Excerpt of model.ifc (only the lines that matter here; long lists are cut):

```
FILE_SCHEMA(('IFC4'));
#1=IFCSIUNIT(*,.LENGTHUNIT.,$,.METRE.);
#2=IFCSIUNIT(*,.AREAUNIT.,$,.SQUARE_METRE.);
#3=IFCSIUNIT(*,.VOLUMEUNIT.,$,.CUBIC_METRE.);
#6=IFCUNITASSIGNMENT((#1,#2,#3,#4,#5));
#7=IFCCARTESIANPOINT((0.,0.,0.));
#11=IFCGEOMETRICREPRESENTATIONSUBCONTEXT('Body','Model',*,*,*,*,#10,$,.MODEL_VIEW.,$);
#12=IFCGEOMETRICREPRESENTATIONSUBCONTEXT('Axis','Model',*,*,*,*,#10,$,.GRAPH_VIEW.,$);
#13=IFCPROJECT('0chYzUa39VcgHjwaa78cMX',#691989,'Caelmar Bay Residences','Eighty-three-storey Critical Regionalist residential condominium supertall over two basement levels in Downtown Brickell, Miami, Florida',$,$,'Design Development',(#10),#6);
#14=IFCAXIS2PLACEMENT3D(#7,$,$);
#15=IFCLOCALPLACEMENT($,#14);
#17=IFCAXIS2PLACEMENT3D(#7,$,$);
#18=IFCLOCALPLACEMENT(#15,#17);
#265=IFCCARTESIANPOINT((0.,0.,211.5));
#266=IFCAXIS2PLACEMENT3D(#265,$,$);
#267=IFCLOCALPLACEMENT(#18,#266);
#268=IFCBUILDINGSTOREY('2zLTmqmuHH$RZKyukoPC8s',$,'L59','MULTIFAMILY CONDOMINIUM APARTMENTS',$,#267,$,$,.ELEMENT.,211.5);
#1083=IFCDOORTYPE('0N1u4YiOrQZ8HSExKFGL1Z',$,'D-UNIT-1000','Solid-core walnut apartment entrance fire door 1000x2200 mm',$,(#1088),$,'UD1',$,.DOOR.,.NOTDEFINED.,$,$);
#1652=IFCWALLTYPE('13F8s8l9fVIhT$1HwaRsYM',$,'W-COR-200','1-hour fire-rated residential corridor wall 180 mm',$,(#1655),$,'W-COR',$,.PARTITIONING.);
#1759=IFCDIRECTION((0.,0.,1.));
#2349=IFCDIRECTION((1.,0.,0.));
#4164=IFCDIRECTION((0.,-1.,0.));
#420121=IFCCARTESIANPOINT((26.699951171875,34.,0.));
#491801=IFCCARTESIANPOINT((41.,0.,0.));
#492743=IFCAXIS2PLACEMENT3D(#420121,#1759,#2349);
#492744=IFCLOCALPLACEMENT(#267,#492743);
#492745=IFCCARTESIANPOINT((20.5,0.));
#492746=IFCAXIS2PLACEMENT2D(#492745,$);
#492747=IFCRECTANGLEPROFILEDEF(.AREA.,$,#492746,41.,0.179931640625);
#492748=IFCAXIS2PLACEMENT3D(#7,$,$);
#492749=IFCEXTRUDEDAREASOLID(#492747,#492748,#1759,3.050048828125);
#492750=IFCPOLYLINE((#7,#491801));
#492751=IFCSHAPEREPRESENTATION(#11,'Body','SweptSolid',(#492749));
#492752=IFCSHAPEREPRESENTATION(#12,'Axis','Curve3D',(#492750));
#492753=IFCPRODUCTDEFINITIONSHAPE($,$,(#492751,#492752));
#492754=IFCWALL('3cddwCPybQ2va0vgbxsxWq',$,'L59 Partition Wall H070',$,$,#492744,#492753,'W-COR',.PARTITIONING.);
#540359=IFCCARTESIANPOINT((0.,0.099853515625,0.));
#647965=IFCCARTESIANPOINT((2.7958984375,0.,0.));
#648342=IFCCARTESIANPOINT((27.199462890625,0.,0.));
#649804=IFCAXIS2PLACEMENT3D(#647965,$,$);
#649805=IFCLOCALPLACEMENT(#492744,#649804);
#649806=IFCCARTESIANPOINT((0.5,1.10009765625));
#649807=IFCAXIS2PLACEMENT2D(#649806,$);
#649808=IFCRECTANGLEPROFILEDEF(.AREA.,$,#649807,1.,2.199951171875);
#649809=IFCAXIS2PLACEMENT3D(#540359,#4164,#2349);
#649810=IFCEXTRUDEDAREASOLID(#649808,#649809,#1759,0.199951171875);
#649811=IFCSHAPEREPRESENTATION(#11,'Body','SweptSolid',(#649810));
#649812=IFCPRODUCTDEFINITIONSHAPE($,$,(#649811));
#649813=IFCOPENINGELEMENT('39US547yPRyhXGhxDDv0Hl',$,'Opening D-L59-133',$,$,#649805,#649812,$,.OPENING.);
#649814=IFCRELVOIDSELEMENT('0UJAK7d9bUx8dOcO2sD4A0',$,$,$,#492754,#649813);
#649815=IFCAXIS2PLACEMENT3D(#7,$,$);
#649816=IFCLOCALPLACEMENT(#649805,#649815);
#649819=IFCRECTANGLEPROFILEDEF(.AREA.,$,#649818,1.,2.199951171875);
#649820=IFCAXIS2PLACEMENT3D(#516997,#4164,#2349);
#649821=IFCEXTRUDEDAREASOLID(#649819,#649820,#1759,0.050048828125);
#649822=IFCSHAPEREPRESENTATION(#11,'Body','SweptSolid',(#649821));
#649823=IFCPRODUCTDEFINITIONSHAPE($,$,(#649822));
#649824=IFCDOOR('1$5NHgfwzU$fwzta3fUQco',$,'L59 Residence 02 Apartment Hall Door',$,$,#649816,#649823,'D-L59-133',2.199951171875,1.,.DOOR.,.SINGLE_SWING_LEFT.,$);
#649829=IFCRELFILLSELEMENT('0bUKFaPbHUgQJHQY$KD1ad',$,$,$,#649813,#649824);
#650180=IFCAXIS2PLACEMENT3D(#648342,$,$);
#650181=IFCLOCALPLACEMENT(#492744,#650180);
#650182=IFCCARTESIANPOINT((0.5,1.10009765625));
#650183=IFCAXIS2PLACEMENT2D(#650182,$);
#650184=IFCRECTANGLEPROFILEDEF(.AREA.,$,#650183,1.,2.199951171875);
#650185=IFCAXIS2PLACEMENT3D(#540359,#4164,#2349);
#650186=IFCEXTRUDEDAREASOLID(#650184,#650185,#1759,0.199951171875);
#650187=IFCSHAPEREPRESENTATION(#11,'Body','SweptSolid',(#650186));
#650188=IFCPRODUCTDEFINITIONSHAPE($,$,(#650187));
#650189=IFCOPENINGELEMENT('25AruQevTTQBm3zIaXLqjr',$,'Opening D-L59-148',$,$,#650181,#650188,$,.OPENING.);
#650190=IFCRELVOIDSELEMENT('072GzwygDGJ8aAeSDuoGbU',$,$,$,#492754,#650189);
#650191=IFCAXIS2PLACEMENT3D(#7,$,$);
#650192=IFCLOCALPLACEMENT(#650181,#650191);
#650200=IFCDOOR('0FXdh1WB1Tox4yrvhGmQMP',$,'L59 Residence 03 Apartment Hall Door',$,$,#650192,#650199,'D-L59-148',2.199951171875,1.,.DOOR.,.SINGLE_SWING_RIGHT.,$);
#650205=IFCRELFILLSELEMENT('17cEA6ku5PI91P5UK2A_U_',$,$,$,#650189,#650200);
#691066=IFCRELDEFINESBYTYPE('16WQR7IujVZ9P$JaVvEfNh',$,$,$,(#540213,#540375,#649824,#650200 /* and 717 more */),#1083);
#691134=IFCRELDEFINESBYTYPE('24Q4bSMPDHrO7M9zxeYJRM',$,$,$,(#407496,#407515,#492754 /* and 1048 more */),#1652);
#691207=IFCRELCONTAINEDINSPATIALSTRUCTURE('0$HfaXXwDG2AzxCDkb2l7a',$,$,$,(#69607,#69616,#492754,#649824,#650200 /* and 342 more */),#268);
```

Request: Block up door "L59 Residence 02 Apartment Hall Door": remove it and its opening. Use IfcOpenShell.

```python
import ifcopenshell
import ifcopenshell.api.feature
import ifcopenshell.api.root
import ifcopenshell.geom
import ifcopenshell.util.shape

model = ifcopenshell.open("model.ifc")
settings = ifcopenshell.geom.settings()


def volume(element):
    """Net volume in cubic metres, openings subtracted."""
    shape = ifcopenshell.geom.create_shape(settings, element)
    return ifcopenshell.util.shape.get_volume(shape.geometry)


door = model.by_guid("1$5NHgfwzU$fwzta3fUQco")
opening = door.FillsVoids[0].RelatingOpeningElement
wall = opening.VoidsElements[0].RelatingBuildingElement
before = volume(wall)

ifcopenshell.api.root.remove_product(model, product=door)
ifcopenshell.api.feature.remove_feature(model, feature=opening)

after = volume(wall)

print(f"wall volume {before:.3f} -> {after:.3f} m3")

model.write("model-out.ifc")
```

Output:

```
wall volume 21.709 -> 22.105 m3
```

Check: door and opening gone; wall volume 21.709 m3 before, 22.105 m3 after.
